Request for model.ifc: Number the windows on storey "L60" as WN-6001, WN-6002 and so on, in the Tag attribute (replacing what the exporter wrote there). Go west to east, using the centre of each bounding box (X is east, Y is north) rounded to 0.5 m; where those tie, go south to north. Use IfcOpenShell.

First a look at what the model holds.

```python
import ifcopenshell
import ifcopenshell.util.element
import ifcopenshell.util.placement

model = ifcopenshell.open("model.ifc")
print(model.schema)
storey = next(s for s in model.by_type("IfcBuildingStorey") if s.Name == "L60")
windows = [e for e in ifcopenshell.util.element.get_decomposition(storey) if e.is_a("IfcWindow")]
for e in sorted(windows, key=lambda e: e.id()):
    origin = ifcopenshell.util.placement.get_local_placement(e.ObjectPlacement)[:3, 3]
    print(e.id(), e.Tag, e.Name, origin.round(2) + 0.0, sep=" | ")
```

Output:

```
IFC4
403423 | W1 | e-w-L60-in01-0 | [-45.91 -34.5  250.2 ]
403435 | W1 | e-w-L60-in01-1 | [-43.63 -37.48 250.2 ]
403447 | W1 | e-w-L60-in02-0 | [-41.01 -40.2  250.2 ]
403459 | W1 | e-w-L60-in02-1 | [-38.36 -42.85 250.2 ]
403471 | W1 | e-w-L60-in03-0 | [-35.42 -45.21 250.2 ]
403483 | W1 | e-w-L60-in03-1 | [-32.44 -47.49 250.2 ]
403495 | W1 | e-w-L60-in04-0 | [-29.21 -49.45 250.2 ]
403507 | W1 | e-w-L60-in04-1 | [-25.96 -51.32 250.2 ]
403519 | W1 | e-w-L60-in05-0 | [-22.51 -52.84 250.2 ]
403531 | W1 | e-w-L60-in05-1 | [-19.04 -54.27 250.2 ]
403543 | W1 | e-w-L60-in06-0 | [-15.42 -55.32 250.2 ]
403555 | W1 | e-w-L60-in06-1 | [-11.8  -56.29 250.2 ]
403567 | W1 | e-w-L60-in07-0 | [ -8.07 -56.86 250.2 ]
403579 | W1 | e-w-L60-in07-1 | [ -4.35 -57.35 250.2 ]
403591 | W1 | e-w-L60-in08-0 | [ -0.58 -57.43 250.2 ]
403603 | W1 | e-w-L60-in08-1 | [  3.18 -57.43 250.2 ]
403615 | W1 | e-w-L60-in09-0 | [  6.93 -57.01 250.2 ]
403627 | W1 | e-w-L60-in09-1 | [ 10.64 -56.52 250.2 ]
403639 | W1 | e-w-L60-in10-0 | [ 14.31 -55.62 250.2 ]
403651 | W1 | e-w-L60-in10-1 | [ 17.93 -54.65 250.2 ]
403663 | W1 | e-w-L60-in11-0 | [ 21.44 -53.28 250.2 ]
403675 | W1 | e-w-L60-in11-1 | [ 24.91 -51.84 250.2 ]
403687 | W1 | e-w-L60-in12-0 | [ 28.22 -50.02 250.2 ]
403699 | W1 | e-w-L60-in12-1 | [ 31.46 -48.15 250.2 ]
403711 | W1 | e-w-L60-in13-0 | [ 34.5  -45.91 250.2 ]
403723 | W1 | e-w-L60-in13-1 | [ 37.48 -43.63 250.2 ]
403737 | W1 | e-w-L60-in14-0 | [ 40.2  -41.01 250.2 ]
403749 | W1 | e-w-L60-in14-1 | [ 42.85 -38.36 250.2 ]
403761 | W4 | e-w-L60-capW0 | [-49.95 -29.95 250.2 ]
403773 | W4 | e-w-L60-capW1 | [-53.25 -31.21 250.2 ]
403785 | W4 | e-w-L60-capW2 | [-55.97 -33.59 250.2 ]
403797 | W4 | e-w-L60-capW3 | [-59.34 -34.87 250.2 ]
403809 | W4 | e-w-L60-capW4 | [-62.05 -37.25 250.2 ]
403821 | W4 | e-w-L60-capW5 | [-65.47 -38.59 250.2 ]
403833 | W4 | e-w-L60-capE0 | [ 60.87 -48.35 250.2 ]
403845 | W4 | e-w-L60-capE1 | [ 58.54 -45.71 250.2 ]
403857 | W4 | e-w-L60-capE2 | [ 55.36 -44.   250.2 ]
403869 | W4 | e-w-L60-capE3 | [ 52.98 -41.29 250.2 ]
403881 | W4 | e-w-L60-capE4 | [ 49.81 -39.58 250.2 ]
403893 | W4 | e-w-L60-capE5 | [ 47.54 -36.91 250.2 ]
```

```python
import ifcopenshell
import ifcopenshell.geom
import ifcopenshell.util.element
import ifcopenshell.util.shape

model = ifcopenshell.open("model.ifc")
settings = ifcopenshell.geom.settings()
settings.set("use-world-coords", True)


def centre(element):
    shape = ifcopenshell.geom.create_shape(settings, element)
    return ifcopenshell.util.shape.get_bbox_centroid(shape.geometry)


storey = next(s for s in model.by_type("IfcBuildingStorey") if s.Name == "L60")
windows = [e for e in ifcopenshell.util.element.get_decomposition(storey) if e.is_a("IfcWindow")]

# Insertion points can sit at a corner or the storey origin, so sort by the geometry (in metres).
centres = {e: centre(e) for e in windows}
windows.sort(key=lambda e: (round(centres[e][0] / 0.5), centres[e][1]))

for i, e in enumerate(windows, start=1):
    number = f"WN-60{i:02d}"
    e.Tag = number
    print(e.id(), number)

model.write("model_edited.ifc")
```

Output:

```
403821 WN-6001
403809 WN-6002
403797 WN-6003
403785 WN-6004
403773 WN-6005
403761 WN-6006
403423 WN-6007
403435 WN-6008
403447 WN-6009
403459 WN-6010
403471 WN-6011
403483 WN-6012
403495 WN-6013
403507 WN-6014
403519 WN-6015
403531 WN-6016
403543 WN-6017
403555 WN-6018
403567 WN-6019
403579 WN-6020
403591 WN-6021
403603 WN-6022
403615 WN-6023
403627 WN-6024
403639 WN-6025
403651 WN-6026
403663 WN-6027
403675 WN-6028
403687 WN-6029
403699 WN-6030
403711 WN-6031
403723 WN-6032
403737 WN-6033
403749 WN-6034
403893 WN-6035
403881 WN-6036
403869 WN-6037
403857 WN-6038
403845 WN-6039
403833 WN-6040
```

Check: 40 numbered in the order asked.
